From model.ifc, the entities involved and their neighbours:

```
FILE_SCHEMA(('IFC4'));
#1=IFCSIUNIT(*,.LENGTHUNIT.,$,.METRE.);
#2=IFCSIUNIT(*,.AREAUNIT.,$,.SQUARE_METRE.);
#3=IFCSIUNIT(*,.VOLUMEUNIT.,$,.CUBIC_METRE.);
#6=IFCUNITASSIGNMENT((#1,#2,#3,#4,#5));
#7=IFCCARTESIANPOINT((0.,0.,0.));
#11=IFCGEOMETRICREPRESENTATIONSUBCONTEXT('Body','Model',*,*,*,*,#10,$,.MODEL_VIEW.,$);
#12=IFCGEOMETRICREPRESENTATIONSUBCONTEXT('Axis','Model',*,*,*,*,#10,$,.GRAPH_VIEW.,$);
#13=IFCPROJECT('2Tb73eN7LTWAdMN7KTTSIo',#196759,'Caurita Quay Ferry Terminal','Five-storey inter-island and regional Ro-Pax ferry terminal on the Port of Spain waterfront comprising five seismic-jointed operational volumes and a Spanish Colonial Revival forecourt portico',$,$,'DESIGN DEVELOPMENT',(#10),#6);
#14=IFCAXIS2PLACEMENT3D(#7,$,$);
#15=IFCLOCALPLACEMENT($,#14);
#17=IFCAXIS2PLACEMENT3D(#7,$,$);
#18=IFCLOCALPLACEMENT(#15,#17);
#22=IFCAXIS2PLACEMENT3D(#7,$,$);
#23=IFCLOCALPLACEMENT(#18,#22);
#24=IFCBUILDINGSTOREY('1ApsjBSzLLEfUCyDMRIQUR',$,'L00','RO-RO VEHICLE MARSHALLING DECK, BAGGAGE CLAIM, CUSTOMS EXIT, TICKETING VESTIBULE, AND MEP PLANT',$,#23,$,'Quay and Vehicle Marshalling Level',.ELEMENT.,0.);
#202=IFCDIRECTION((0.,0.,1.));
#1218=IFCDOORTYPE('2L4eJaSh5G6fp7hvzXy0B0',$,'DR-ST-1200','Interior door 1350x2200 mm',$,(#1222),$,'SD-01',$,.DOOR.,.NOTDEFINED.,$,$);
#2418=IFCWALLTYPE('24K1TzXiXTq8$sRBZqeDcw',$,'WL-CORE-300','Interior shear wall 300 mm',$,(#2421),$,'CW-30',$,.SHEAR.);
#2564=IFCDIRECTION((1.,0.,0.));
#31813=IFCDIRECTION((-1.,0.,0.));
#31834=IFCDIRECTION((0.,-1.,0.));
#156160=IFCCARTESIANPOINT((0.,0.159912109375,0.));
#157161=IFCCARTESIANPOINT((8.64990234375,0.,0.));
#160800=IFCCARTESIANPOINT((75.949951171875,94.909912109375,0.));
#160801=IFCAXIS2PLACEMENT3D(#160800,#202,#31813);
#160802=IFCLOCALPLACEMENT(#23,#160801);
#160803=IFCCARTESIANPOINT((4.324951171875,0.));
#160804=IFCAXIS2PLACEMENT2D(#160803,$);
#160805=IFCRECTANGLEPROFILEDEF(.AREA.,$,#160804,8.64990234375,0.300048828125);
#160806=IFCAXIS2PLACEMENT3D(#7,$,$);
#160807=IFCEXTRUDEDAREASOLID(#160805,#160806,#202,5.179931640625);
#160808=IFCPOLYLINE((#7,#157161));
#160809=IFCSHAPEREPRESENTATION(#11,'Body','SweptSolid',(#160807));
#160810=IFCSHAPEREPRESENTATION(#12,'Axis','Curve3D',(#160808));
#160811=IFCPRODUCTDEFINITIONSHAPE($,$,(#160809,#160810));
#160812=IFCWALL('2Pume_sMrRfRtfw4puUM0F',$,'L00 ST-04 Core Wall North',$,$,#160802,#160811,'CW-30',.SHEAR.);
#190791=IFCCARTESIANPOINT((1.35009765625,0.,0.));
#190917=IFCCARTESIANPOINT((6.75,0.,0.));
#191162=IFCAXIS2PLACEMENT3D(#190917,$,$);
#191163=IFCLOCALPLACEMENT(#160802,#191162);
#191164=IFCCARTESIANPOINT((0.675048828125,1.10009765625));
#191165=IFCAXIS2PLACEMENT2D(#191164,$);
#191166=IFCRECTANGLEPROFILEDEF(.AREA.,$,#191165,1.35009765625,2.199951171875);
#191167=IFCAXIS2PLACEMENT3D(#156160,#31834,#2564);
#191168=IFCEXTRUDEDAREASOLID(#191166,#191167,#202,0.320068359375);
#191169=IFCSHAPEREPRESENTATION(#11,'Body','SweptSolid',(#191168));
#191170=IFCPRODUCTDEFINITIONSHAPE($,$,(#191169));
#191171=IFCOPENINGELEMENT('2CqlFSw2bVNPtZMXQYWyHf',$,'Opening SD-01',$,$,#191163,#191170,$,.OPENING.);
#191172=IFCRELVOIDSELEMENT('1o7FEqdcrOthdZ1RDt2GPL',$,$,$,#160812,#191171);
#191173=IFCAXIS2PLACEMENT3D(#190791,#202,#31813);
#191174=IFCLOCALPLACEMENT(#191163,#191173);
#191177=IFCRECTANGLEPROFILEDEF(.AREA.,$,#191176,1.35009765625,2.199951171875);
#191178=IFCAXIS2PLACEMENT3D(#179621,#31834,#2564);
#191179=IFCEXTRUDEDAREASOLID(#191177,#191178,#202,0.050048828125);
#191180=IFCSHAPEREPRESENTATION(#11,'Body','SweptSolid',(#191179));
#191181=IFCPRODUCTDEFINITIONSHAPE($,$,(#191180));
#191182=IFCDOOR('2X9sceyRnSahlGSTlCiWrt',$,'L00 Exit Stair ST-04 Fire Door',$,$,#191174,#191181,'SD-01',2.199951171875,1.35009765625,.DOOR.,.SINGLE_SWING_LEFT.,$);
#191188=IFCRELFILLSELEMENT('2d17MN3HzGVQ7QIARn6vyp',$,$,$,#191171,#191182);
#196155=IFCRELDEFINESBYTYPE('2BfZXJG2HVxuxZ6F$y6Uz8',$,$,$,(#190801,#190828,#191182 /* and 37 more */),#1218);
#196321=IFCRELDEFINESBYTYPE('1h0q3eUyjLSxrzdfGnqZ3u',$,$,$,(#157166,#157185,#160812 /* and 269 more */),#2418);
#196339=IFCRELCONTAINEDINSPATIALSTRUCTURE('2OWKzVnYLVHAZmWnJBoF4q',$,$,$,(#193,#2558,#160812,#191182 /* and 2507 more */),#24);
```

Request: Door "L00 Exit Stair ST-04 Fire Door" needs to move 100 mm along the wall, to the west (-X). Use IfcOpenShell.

```python
import ifcopenshell
import ifcopenshell.api.geometry
import ifcopenshell.util.placement
import ifcopenshell.util.unit

model = ifcopenshell.open("model.ifc")
unit_scale = ifcopenshell.util.unit.calculate_unit_scale(model)

door = model.by_guid("2X9sceyRnSahlGSTlCiWrt")
opening = door.FillsVoids[0].RelatingOpeningElement
wall = opening.VoidsElements[0].RelatingBuildingElement

wall_matrix = ifcopenshell.util.placement.get_local_placement(wall.ObjectPlacement)
shift = wall_matrix[:3, 0] * 0.1 / unit_scale
before = ifcopenshell.util.placement.get_local_placement(door.ObjectPlacement)[:3, 3].copy()

# The door is placed relative to its opening, so it follows when the opening moves.
matrix = ifcopenshell.util.placement.get_local_placement(opening.ObjectPlacement)
matrix[:3, 3] += shift
ifcopenshell.api.geometry.edit_object_placement(
    model, product=opening, matrix=matrix, is_si=False, should_transform_children=True
)

after = ifcopenshell.util.placement.get_local_placement(door.ObjectPlacement)[:3, 3]
print("door moved by", (after - before).round(3) + 0.0)

model.write("model_v2.ifc")
```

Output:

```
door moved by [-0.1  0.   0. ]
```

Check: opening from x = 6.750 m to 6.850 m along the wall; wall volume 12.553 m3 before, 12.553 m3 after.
